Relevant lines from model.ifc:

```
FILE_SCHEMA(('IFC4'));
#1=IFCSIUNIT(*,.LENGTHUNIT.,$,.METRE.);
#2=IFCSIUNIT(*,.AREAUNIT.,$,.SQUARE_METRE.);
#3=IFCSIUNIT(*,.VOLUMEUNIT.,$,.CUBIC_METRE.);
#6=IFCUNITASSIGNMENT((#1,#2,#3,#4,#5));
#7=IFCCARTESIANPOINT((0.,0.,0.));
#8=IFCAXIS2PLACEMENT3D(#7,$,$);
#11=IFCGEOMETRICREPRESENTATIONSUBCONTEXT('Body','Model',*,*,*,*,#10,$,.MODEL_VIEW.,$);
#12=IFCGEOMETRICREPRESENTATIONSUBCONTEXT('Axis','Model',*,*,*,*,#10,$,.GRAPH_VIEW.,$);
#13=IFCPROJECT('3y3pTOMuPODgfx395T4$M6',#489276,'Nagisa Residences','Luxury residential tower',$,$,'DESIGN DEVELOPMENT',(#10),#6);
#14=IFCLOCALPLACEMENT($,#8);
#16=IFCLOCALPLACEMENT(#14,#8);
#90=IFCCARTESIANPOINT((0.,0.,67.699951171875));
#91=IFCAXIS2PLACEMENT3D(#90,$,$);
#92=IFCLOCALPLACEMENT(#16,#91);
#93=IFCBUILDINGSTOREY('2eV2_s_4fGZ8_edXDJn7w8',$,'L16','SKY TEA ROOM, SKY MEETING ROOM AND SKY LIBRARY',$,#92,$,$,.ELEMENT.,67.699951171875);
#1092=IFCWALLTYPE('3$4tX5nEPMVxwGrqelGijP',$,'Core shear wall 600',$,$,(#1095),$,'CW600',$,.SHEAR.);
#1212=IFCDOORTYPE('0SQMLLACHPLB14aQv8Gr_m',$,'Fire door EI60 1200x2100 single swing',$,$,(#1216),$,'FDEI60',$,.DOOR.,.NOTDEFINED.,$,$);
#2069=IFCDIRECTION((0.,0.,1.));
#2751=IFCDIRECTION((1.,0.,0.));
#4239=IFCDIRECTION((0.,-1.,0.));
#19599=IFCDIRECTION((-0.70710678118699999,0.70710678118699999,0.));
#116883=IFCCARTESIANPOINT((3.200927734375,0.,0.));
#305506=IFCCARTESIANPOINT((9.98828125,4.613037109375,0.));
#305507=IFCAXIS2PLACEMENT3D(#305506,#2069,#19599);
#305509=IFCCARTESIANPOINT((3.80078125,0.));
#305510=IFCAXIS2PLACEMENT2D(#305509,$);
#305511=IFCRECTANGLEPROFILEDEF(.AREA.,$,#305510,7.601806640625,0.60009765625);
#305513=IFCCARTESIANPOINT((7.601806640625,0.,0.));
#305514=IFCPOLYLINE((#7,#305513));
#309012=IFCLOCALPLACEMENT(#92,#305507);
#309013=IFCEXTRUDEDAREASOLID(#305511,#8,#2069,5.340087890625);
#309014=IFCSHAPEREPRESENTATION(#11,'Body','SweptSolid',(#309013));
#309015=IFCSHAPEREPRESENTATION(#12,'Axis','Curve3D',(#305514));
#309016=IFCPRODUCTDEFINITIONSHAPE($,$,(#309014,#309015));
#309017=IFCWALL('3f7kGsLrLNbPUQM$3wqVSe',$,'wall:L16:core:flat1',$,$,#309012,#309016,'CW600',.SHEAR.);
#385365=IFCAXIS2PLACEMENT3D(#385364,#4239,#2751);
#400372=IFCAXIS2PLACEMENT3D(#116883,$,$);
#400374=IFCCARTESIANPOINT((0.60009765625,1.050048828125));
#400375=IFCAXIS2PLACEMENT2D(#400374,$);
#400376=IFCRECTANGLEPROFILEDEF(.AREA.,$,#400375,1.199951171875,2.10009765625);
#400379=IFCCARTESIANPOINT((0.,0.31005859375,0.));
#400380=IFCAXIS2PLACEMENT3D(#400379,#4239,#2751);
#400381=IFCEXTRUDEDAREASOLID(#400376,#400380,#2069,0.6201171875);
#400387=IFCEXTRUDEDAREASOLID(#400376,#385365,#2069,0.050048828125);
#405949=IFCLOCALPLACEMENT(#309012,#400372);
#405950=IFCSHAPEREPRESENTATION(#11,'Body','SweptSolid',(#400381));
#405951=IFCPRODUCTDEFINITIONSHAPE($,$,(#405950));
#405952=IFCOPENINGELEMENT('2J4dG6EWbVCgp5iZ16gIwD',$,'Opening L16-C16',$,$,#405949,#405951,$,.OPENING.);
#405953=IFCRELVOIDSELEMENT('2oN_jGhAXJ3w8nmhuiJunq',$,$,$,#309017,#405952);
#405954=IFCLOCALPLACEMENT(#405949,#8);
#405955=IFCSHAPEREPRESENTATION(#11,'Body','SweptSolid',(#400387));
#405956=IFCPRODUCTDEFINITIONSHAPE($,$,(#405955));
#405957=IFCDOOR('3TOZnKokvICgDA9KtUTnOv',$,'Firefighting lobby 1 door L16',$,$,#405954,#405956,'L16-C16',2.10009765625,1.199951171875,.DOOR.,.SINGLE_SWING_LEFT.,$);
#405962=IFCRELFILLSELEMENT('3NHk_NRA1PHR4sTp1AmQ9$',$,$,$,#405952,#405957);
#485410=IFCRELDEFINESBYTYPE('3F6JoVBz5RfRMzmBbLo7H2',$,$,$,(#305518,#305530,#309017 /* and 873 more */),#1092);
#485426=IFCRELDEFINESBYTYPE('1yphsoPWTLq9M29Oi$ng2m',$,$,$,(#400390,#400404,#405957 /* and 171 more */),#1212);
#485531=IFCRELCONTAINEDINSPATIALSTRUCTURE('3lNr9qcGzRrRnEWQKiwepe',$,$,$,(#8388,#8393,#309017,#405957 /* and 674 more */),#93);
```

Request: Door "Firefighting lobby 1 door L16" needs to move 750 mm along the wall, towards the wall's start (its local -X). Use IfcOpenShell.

```python
import ifcopenshell
import ifcopenshell.api.geometry
import ifcopenshell.util.placement
import ifcopenshell.util.unit

model = ifcopenshell.open("model.ifc")
unit_scale = ifcopenshell.util.unit.calculate_unit_scale(model)

door = model.by_guid("3TOZnKokvICgDA9KtUTnOv")
opening = door.FillsVoids[0].RelatingOpeningElement
wall = opening.VoidsElements[0].RelatingBuildingElement

wall_matrix = ifcopenshell.util.placement.get_local_placement(wall.ObjectPlacement)
shift = wall_matrix[:3, 0] * -0.75 / unit_scale
before = ifcopenshell.util.placement.get_local_placement(door.ObjectPlacement)[:3, 3].copy()

# The door is placed relative to its opening, so it follows when the opening moves.
matrix = ifcopenshell.util.placement.get_local_placement(opening.ObjectPlacement)
matrix[:3, 3] += shift
ifcopenshell.api.geometry.edit_object_placement(
    model, product=opening, matrix=matrix, is_si=False, should_transform_children=True
)

after = ifcopenshell.util.placement.get_local_placement(door.ObjectPlacement)[:3, 3]
print("door moved by", (after - before).round(3) + 0.0)

model.write("model_edited.ifc")
```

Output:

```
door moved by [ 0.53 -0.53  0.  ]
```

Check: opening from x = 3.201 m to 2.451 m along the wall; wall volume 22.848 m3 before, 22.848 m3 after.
